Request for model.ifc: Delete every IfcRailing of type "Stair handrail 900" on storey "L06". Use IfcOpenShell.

First a look at what the model holds.

```python
import ifcopenshell
import ifcopenshell.util.element

model = ifcopenshell.open("model.ifc")
print(model.schema)
storey = next(s for s in model.by_type("IfcBuildingStorey") if s.Name == "L06")
railings = [e for e in ifcopenshell.util.element.get_decomposition(storey) if e.is_a("IfcRailing")]
seen = {}
for e in railings:
    element_type = ifcopenshell.util.element.get_type(e)
    name = element_type.Name if element_type not in (None, e) else None
    seen[name] = seen.get(name, 0) + 1
for name, count in sorted(seen.items(), key=str):
    print(count, "x", name)
```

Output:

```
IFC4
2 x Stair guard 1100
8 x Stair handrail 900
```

```python
import ifcopenshell
import ifcopenshell.api.root
import ifcopenshell.util.element

model = ifcopenshell.open("model.ifc")

storey = next(s for s in model.by_type("IfcBuildingStorey") if s.Name == "L06")
railings = [e for e in ifcopenshell.util.element.get_decomposition(storey) if e.is_a("IfcRailing")]
targets = [e for e in railings if (t := ifcopenshell.util.element.get_type(e)) not in (None, e) and t.Name == "Stair handrail 900"]

for e in targets:
    ifcopenshell.api.root.remove_product(model, product=e)
print(len(targets), "removed")

model.write("model_rev.ifc")
```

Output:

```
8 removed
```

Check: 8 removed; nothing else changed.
